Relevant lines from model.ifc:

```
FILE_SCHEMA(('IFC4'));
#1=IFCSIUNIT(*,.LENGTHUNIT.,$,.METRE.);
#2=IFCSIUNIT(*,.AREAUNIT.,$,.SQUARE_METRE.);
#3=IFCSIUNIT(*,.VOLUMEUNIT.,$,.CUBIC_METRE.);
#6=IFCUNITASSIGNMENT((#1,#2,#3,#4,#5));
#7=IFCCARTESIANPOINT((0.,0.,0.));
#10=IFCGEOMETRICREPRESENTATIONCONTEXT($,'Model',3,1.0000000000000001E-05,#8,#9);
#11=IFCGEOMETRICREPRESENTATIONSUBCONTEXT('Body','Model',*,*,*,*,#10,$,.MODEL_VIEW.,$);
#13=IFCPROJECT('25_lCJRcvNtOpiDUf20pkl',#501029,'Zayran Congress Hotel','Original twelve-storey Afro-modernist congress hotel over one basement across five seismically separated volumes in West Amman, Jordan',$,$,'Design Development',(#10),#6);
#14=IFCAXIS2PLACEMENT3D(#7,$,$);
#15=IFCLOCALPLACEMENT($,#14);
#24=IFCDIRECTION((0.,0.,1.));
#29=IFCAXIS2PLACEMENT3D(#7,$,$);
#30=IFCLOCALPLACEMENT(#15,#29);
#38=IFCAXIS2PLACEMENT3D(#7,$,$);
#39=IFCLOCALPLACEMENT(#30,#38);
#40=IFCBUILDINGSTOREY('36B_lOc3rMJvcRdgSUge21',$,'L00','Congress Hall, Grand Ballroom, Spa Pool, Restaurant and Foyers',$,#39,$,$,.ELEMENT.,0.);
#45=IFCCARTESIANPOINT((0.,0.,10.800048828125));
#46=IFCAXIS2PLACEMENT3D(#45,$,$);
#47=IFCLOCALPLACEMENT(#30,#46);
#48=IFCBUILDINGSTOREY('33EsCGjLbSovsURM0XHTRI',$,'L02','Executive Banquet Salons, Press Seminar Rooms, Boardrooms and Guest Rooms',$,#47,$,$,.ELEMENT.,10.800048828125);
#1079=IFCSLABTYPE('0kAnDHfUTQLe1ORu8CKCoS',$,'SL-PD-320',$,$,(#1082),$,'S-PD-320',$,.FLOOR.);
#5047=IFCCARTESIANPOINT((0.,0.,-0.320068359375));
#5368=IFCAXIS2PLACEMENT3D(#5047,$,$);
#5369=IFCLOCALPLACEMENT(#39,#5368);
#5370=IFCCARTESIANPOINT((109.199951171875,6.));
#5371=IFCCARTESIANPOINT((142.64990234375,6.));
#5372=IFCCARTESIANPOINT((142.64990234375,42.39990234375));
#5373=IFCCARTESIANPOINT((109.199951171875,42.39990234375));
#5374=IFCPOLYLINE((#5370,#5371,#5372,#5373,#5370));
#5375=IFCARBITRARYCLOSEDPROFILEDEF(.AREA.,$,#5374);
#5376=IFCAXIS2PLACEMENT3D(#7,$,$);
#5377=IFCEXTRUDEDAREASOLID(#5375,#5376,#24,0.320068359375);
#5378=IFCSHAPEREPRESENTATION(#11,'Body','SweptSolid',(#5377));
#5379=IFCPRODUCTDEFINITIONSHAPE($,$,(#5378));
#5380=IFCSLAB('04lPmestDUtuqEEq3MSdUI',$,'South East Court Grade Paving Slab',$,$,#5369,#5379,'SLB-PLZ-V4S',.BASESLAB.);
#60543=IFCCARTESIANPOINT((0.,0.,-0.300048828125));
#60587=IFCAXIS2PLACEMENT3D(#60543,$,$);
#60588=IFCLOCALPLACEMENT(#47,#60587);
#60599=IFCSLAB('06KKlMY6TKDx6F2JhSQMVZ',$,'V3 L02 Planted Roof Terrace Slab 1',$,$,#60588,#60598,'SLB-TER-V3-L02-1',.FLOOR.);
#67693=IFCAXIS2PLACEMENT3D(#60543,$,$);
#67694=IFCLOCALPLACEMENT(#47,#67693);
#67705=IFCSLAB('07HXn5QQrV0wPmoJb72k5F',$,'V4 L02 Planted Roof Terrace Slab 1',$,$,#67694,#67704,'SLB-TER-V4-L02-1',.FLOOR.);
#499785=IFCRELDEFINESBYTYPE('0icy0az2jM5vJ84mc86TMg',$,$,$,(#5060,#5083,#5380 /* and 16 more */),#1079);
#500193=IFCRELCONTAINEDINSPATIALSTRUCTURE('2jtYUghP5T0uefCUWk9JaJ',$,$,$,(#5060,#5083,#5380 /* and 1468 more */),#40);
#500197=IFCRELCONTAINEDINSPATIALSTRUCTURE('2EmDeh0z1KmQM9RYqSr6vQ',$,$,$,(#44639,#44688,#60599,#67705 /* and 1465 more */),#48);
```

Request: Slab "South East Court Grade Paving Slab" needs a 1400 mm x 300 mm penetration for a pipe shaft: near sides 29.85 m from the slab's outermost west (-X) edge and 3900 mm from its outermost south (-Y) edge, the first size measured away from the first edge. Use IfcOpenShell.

```python
import numpy as np
import ifcopenshell
import ifcopenshell.api.feature
import ifcopenshell.api.geometry
import ifcopenshell.api.root
import ifcopenshell.geom
import ifcopenshell.util.placement
import ifcopenshell.util.representation
import ifcopenshell.util.shape
import ifcopenshell.util.unit

model = ifcopenshell.open("model.ifc")
unit_scale = ifcopenshell.util.unit.calculate_unit_scale(model)
settings = ifcopenshell.geom.settings()


def volume(element):
    """Net volume in cubic metres, openings subtracted."""
    shape = ifcopenshell.geom.create_shape(settings, element)
    return ifcopenshell.util.shape.get_volume(shape.geometry)


slab = model.by_guid("04lPmestDUtuqEEq3MSdUI")
before = volume(slab)

# Extent in the slab's own axes, in metres. The edges named are its -X and -Y sides.
slab_shape = ifcopenshell.geom.create_shape(settings, slab)
vertices = ifcopenshell.util.shape.get_vertices(slab_shape.geometry)
x_min, y_min, bottom = vertices.min(axis=0)
top = vertices[:, 2].max()

opening = ifcopenshell.api.root.create_entity(model, ifc_class="IfcOpeningElement", name="Pipe shaft opening", predefined_type="OPENING")
context = ifcopenshell.util.representation.get_context(model, "Model", "Body", "MODEL_VIEW")
width, depth = 1.4, 0.3
outline = [(0.0, 0.0), (width, 0.0), (width, depth), (0.0, depth), (0.0, 0.0)]
# Overshoot both faces by 50 mm so the cut is clean.
shape = ifcopenshell.api.geometry.add_slab_representation(
    model, context=context, depth=top - bottom + 0.1, polyline=outline
)
ifcopenshell.api.geometry.assign_representation(model, product=opening, representation=shape)

matrix = ifcopenshell.util.placement.get_local_placement(slab.ObjectPlacement)
matrix[:, 3] = matrix @ np.append(np.array([x_min + 29.85, y_min + 3.9, bottom - 0.05]) / unit_scale, 1.0)
ifcopenshell.api.geometry.edit_object_placement(model, product=opening, matrix=matrix, is_si=False)
ifcopenshell.api.feature.add_feature(model, feature=opening, element=slab)

after = volume(slab)

print(f"slab volume {before:.3f} -> {after:.3f} m3")

model.write("model_updated.ifc")
```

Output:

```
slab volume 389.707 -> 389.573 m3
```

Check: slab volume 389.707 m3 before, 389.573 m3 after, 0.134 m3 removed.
